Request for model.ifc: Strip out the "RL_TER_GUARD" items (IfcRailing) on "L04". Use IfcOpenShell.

First a look at what the model holds.

```python
import ifcopenshell
import ifcopenshell.util.element

model = ifcopenshell.open("model.ifc")
print(model.schema)
storey = next(s for s in model.by_type("IfcBuildingStorey") if s.Name == "L04")
railings = [e for e in ifcopenshell.util.element.get_decomposition(storey) if e.is_a("IfcRailing")]
seen = {}
for e in railings:
    element_type = ifcopenshell.util.element.get_type(e)
    name = element_type.Name if element_type not in (None, e) else None
    seen[name] = seen.get(name, 0) + 1
for name, count in sorted(seen.items(), key=str):
    print(count, "x", name)
```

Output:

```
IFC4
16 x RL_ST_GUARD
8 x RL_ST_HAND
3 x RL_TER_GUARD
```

```python
import ifcopenshell
import ifcopenshell.api.root
import ifcopenshell.util.element

model = ifcopenshell.open("model.ifc")

storey = next(s for s in model.by_type("IfcBuildingStorey") if s.Name == "L04")
railings = [e for e in ifcopenshell.util.element.get_decomposition(storey) if e.is_a("IfcRailing")]
targets = [e for e in railings if (t := ifcopenshell.util.element.get_type(e)) not in (None, e) and t.Name == "RL_TER_GUARD"]

for e in targets:
    ifcopenshell.api.root.remove_product(model, product=e)
print(len(targets), "removed")

model.write("model_updated.ifc")
```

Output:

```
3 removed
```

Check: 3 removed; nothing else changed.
